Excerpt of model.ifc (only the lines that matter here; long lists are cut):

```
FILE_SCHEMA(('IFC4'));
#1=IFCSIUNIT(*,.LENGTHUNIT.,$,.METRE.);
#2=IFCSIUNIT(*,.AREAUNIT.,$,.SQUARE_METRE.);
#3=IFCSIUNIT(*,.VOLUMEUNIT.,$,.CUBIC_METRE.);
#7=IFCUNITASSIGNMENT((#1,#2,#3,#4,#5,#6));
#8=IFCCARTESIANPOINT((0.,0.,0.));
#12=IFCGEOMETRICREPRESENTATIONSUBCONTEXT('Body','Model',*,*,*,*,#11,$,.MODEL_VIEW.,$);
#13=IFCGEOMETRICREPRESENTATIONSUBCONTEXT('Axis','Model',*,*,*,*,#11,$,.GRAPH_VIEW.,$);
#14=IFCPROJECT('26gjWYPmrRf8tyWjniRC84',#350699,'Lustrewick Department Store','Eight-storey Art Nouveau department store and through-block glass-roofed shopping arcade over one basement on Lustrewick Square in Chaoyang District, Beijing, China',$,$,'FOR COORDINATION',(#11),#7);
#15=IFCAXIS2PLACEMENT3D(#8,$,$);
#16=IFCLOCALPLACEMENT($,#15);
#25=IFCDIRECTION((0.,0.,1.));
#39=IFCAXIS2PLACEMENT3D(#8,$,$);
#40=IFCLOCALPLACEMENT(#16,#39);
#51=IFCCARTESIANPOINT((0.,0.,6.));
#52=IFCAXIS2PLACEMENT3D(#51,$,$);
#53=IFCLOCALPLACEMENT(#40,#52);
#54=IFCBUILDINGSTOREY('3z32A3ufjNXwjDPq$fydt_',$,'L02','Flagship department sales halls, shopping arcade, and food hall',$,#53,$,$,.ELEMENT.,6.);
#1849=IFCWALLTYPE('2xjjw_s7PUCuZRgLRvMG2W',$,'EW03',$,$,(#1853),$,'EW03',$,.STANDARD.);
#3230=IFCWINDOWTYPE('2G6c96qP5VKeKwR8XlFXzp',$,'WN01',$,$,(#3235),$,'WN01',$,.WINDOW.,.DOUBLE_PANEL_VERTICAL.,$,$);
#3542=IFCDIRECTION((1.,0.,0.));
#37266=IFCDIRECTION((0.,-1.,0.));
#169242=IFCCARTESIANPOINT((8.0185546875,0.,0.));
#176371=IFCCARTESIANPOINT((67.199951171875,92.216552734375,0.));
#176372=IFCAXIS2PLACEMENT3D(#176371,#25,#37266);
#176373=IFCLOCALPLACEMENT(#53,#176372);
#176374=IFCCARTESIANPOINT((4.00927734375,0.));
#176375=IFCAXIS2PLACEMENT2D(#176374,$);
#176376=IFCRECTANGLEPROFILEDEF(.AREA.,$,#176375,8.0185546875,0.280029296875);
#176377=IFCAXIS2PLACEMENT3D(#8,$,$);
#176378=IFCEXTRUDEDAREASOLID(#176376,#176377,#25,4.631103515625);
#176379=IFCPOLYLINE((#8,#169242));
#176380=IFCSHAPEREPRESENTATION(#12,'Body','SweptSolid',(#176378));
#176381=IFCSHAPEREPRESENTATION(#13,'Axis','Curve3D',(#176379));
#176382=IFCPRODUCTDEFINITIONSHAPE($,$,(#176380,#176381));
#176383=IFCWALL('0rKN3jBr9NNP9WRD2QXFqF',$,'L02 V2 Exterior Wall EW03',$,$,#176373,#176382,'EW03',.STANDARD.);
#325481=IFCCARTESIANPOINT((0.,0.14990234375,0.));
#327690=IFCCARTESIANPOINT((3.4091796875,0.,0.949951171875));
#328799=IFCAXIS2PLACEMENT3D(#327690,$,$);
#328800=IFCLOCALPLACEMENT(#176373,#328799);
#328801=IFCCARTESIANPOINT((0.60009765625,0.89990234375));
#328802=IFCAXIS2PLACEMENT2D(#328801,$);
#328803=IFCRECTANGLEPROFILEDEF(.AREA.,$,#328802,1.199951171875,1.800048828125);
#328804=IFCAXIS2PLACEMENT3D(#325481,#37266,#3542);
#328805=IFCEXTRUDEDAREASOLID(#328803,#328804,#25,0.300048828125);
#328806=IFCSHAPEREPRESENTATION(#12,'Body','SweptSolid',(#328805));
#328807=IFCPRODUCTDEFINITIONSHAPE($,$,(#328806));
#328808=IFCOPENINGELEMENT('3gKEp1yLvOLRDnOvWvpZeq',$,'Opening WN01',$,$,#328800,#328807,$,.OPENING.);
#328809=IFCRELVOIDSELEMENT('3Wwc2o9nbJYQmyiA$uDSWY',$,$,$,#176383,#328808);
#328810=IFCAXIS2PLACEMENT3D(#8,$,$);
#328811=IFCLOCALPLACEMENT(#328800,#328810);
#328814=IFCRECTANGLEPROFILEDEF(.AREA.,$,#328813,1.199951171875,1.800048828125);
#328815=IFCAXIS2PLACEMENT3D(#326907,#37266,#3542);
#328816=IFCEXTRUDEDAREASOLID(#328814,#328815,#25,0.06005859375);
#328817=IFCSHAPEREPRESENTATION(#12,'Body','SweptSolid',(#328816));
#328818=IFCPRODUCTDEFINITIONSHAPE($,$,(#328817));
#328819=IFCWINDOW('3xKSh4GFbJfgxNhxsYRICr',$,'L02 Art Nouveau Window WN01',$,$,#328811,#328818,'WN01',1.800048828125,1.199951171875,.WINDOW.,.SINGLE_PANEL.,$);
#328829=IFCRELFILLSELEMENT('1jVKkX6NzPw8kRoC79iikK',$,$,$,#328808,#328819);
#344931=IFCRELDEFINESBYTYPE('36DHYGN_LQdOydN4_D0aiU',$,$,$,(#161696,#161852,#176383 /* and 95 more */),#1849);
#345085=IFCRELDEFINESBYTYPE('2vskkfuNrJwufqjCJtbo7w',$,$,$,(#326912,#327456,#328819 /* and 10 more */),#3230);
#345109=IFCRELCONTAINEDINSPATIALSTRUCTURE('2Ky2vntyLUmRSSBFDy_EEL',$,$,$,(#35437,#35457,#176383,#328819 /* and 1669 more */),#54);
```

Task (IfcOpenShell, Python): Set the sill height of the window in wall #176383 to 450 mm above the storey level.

```python
import numpy as np
import ifcopenshell
import ifcopenshell.api.geometry
import ifcopenshell.geom
import ifcopenshell.util.element
import ifcopenshell.util.placement
import ifcopenshell.util.shape
import ifcopenshell.util.unit

model = ifcopenshell.open("model.ifc")
unit_scale = ifcopenshell.util.unit.calculate_unit_scale(model)

window = model.by_guid("3xKSh4GFbJfgxNhxsYRICr")
opening = window.FillsVoids[0].RelatingOpeningElement
storey = ifcopenshell.util.element.get_container(window, ifc_class="IfcBuildingStorey")
level = ifcopenshell.util.placement.get_local_placement(storey.ObjectPlacement)[2, 3]

# The opening's origin need not be at the sill, so measure its lowest point.
shape = ifcopenshell.geom.create_shape(ifcopenshell.geom.settings(), opening)
bottom = ifcopenshell.util.shape.get_shape_bottom_elevation(shape, shape.geometry) / unit_scale
dz = level + 0.45 - bottom

shift = np.array([0.0, 0.0, dz])
# The window is placed relative to its opening, so it follows when the opening moves.
matrix = ifcopenshell.util.placement.get_local_placement(opening.ObjectPlacement)
matrix[:3, 3] += shift
ifcopenshell.api.geometry.edit_object_placement(
    model, product=opening, matrix=matrix, is_si=False, should_transform_children=True
)

print(f"moved by {dz * unit_scale:+.3f} m")

model.write("model_edited.ifc")
```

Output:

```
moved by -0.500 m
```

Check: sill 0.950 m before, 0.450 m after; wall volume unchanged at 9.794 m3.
